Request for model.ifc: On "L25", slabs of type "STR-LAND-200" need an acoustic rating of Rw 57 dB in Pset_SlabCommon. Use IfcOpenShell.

First a look at what the model holds.

```python
import ifcopenshell
import ifcopenshell.util.element

model = ifcopenshell.open("model.ifc")
print(model.schema)
storey = next(s for s in model.by_type("IfcBuildingStorey") if s.Name == "L25")
slabs = [e for e in ifcopenshell.util.element.get_decomposition(storey) if e.is_a("IfcSlab")]
seen = {}
for e in slabs:
    element_type = ifcopenshell.util.element.get_type(e)
    key = (element_type.Name if element_type != e and element_type else None, ifcopenshell.util.element.get_pset(e, "Pset_SlabCommon", "AcousticRating"))
    seen[key] = seen.get(key, 0) + 1
for (name, value), count in sorted(seen.items(), key=str):
    print(count, "x", name, "|", value)
```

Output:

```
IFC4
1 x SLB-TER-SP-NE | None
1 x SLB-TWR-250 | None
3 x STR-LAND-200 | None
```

```python
import ifcopenshell
import ifcopenshell.api.pset
import ifcopenshell.util.element

model = ifcopenshell.open("model.ifc")

storey = next(s for s in model.by_type("IfcBuildingStorey") if s.Name == "L25")
slabs = [e for e in ifcopenshell.util.element.get_decomposition(storey) if e.is_a("IfcSlab")]

count = 0
for e in slabs:
    element_type = ifcopenshell.util.element.get_type(e)
    if element_type in (None, e) or element_type.Name != "STR-LAND-200":
        continue
    found = ifcopenshell.util.element.get_pset(e, "Pset_SlabCommon", should_inherit=False)
    if found:
        pset = model.by_id(found["id"])
        if len(ifcopenshell.util.element.get_elements_by_pset(pset)) > 1:
            pset = ifcopenshell.api.pset.unshare_pset(model, products=[e], pset=pset)[0]
    else:
        pset = ifcopenshell.api.pset.add_pset(model, product=e, name="Pset_SlabCommon")
    ifcopenshell.api.pset.edit_pset(model, pset=pset, properties={"AcousticRating": "Rw 57 dB"})
    count += 1

print(count, "slabs updated")

model.write("model_edited.ifc")
```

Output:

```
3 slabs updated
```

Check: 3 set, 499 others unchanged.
